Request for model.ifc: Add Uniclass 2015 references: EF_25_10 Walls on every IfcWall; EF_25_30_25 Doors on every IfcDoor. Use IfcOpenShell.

First a look at what the model holds.

```python
import ifcopenshell

model = ifcopenshell.open("model.ifc")
print(model.schema)
print("classifications:", [c.Name for c in model.by_type("IfcClassification")])
for ifc_class in ("IfcDoor", "IfcRoof", "IfcStair", "IfcWall", "IfcWindow"):
    print(ifc_class, len(model.by_type(ifc_class)))
```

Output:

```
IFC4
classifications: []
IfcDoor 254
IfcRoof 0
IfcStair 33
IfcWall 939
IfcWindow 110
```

```python
import ifcopenshell
import ifcopenshell.api.classification

model = ifcopenshell.open("model.ifc")

system = ifcopenshell.api.classification.add_classification(model, classification="Uniclass 2015")

codes = {
    "IfcWall": ("EF_25_10", "Walls"),
    "IfcDoor": ("EF_25_30_25", "Doors"),
}
for ifc_class, (code, name) in codes.items():
    products = model.by_type(ifc_class)
    ifcopenshell.api.classification.add_reference(
        model, products=products, classification=system, identification=code, name=name
    )
    print(code, len(products))

model.write("model_v2.ifc")
```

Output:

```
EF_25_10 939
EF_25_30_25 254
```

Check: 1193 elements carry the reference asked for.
